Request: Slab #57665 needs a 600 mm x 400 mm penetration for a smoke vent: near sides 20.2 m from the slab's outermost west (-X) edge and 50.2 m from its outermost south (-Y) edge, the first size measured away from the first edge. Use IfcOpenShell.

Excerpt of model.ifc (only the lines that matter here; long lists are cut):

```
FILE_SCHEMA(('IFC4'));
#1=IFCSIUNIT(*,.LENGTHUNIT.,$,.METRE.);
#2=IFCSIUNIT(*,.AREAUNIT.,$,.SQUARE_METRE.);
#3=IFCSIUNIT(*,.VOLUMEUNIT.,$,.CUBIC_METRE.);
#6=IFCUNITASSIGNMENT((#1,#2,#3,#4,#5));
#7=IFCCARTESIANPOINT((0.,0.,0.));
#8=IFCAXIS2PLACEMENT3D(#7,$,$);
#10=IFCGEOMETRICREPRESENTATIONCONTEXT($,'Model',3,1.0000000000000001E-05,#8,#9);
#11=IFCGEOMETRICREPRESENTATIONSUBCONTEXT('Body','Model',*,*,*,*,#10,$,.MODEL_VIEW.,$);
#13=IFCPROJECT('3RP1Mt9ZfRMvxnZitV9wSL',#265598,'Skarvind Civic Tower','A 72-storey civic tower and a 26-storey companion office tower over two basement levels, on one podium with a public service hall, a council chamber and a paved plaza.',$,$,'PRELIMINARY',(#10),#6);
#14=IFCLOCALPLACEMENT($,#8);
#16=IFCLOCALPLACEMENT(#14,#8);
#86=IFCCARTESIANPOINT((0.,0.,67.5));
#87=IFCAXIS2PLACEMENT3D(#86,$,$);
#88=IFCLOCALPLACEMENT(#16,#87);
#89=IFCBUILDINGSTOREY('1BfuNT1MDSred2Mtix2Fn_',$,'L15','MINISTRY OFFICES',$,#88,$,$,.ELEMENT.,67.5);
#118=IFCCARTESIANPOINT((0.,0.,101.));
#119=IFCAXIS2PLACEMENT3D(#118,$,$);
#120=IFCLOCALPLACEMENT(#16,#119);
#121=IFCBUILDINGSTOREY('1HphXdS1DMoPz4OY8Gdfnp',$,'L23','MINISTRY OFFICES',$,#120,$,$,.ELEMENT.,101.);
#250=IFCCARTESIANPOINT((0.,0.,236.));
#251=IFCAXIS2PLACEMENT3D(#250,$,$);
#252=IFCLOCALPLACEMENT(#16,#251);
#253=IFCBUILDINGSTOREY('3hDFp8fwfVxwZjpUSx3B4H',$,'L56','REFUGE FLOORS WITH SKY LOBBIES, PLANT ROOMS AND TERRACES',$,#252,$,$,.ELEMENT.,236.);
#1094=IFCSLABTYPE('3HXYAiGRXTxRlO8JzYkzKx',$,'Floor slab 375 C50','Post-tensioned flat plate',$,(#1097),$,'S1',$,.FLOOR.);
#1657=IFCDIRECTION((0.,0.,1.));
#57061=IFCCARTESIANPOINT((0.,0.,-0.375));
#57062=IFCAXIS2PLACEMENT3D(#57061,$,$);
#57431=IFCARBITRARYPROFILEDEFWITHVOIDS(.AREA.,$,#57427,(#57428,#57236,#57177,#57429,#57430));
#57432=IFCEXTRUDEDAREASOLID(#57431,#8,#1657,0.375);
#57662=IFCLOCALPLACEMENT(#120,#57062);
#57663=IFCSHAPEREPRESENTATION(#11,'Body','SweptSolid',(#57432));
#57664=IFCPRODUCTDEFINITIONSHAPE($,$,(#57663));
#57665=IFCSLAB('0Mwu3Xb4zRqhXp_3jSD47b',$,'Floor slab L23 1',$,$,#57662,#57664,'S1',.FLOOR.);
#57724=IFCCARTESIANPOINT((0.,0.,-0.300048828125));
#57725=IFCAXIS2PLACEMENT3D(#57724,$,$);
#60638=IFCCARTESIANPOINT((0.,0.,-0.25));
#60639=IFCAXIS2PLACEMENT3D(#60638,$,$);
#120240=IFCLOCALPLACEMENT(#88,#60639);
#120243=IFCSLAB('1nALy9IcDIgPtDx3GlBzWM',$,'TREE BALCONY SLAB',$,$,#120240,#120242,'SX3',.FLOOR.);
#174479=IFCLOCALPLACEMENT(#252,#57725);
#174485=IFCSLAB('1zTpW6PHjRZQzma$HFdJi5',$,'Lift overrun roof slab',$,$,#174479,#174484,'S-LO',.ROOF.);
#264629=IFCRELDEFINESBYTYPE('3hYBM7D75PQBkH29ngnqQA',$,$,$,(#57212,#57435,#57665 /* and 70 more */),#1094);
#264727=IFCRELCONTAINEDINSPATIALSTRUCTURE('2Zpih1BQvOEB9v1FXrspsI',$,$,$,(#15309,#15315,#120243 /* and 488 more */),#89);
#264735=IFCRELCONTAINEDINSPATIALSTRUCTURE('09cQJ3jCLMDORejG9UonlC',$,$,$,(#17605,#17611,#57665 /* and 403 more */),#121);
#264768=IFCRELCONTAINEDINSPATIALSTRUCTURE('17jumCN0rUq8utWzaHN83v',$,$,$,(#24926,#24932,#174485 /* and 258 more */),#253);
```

```python
import numpy as np
import ifcopenshell
import ifcopenshell.api.feature
import ifcopenshell.api.geometry
import ifcopenshell.api.root
import ifcopenshell.geom
import ifcopenshell.util.placement
import ifcopenshell.util.representation
import ifcopenshell.util.shape
import ifcopenshell.util.unit

model = ifcopenshell.open("model.ifc")
unit_scale = ifcopenshell.util.unit.calculate_unit_scale(model)
settings = ifcopenshell.geom.settings()


def volume(element):
    """Net volume in cubic metres, openings subtracted."""
    shape = ifcopenshell.geom.create_shape(settings, element)
    return ifcopenshell.util.shape.get_volume(shape.geometry)


slab = model.by_guid("0Mwu3Xb4zRqhXp_3jSD47b")
before = volume(slab)

# Extent in the slab's own axes, in metres. The edges named are its -X and -Y sides.
slab_shape = ifcopenshell.geom.create_shape(settings, slab)
vertices = ifcopenshell.util.shape.get_vertices(slab_shape.geometry)
x_min, y_min, bottom = vertices.min(axis=0)
top = vertices[:, 2].max()

opening = ifcopenshell.api.root.create_entity(model, ifc_class="IfcOpeningElement", name="Smoke vent opening", predefined_type="OPENING")
context = ifcopenshell.util.representation.get_context(model, "Model", "Body", "MODEL_VIEW")
width, depth = 0.6, 0.4
outline = [(0.0, 0.0), (width, 0.0), (width, depth), (0.0, depth), (0.0, 0.0)]
# Overshoot both faces by 50 mm so the cut is clean.
shape = ifcopenshell.api.geometry.add_slab_representation(
    model, context=context, depth=top - bottom + 0.1, polyline=outline
)
ifcopenshell.api.geometry.assign_representation(model, product=opening, representation=shape)

matrix = ifcopenshell.util.placement.get_local_placement(slab.ObjectPlacement)
matrix[:, 3] = matrix @ np.append(np.array([x_min + 20.2, y_min + 50.2, bottom - 0.05]) / unit_scale, 1.0)
ifcopenshell.api.geometry.edit_object_placement(model, product=opening, matrix=matrix, is_si=False)
ifcopenshell.api.feature.add_feature(model, feature=opening, element=slab)

after = volume(slab)

print(f"slab volume {before:.3f} -> {after:.3f} m3")

model.write("model_updated.ifc")
```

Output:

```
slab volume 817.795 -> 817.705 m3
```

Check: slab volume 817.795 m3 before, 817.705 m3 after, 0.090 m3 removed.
